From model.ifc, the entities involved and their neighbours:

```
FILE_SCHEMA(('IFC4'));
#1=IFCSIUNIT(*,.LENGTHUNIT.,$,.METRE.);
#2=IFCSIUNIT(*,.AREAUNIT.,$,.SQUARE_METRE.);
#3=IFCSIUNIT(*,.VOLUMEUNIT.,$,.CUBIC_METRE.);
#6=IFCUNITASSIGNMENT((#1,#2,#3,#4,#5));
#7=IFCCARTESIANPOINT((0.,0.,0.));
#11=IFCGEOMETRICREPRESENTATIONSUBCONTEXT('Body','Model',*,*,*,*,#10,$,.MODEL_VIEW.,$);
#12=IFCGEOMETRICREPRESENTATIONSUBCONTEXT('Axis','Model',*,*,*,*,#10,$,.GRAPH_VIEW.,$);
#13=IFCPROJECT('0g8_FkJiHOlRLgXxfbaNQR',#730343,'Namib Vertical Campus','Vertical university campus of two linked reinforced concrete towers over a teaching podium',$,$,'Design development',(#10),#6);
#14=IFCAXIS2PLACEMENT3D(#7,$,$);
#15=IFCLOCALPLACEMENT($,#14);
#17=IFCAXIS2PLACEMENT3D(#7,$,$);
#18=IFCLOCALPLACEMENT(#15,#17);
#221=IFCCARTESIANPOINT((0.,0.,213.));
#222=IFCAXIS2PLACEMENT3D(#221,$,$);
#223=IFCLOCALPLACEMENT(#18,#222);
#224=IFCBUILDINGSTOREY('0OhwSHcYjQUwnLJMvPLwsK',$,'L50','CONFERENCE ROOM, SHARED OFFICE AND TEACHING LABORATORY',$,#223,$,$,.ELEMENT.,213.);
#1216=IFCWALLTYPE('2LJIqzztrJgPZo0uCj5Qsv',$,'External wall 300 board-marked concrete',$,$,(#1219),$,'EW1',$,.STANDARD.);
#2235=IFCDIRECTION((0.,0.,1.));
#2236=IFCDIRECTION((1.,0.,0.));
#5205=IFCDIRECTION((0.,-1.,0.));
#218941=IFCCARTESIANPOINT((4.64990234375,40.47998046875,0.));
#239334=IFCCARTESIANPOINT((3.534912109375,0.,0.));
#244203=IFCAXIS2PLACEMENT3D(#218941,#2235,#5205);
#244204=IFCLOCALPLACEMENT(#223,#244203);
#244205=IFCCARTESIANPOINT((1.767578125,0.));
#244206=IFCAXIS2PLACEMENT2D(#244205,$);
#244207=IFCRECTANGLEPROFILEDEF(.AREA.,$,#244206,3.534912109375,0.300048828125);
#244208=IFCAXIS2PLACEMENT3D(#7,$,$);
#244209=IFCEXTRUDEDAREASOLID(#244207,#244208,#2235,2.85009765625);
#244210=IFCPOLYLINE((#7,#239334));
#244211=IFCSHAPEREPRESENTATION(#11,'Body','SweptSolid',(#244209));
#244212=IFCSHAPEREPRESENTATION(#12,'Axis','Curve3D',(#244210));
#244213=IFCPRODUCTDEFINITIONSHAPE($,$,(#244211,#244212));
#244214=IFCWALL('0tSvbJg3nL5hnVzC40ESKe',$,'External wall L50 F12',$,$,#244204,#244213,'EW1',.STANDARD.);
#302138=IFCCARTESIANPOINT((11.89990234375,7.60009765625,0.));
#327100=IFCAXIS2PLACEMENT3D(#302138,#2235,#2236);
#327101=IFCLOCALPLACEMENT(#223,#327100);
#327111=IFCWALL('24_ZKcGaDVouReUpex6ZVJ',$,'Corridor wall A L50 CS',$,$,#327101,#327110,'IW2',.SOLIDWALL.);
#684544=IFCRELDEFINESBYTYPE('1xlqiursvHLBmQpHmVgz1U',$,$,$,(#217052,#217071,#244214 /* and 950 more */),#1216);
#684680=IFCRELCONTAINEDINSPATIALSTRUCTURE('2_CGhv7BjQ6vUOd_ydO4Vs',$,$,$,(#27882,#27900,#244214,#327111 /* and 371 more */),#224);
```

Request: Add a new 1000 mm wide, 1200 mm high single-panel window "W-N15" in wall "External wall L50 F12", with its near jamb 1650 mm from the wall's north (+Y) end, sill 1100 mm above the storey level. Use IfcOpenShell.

```python
import numpy as np
import ifcopenshell
import ifcopenshell.api.feature
import ifcopenshell.api.geometry
import ifcopenshell.api.root
import ifcopenshell.api.spatial
import ifcopenshell.geom
import ifcopenshell.util.element
import ifcopenshell.util.placement
import ifcopenshell.util.representation
import ifcopenshell.util.shape
import ifcopenshell.util.unit

model = ifcopenshell.open("model.ifc")
unit_scale = ifcopenshell.util.unit.calculate_unit_scale(model)
settings = ifcopenshell.geom.settings()


def volume(element):
    """Net volume in cubic metres, openings subtracted."""
    shape = ifcopenshell.geom.create_shape(settings, element)
    return ifcopenshell.util.shape.get_volume(shape.geometry)


wall = model.by_guid("0tSvbJg3nL5hnVzC40ESKe")
storey = ifcopenshell.util.element.get_container(wall, ifc_class="IfcBuildingStorey")
context = ifcopenshell.util.representation.get_context(model, "Model", "Body", "MODEL_VIEW")
before = volume(wall)

width, height, from_end, sill = 1, 1.2, 1.65, 1.1  # metres

# The wall runs along its own X axis, and the end named is its -X end.
wall_shape = ifcopenshell.geom.create_shape(settings, wall)
x, y, z = ifcopenshell.util.shape.get_vertices(wall_shape.geometry).T
start = x.min() + from_end
face, thickness = float(y.min()), float(y.max() - y.min())
wall_matrix = ifcopenshell.util.placement.get_local_placement(wall.ObjectPlacement)
level = ifcopenshell.util.placement.get_local_placement(storey.ObjectPlacement)[2, 3]


def in_wall(x, y):
    """Placement at x, y metres in the wall's axes, at sill height."""
    matrix = wall_matrix.copy()
    matrix[:, 3] = wall_matrix @ np.array([x / unit_scale, y / unit_scale, 0.0, 1.0])
    matrix[2, 3] = level + sill / unit_scale
    return matrix


# Opening: a box that overshoots both wall faces by 50 mm.
opening = ifcopenshell.api.root.create_entity(model, ifc_class="IfcOpeningElement", predefined_type="OPENING")
box = ifcopenshell.api.geometry.add_wall_representation(
    model, context=context, length=width, height=height, thickness=thickness + 0.1
)
ifcopenshell.api.geometry.assign_representation(model, product=opening, representation=box)
ifcopenshell.api.geometry.edit_object_placement(model, product=opening, matrix=in_wall(start, face - 0.05), is_si=False)
ifcopenshell.api.feature.add_feature(model, feature=opening, element=wall)

window = ifcopenshell.api.root.create_entity(model, ifc_class="IfcWindow", name="W-N15", predefined_type="WINDOW")
window.OverallWidth, window.OverallHeight = width / unit_scale, height / unit_scale
window.PartitioningType = "SINGLE_PANEL"
body = ifcopenshell.api.geometry.add_window_representation(
    model,
    context=context,
    overall_width=window.OverallWidth,
    overall_height=window.OverallHeight,
    partition_type="SINGLE_PANEL",
)
ifcopenshell.api.geometry.assign_representation(model, product=window, representation=body)
ifcopenshell.api.spatial.assign_container(model, products=[window], relating_structure=storey)
ifcopenshell.api.feature.add_filling(model, opening=opening, element=window)

# Centre the window in the wall's thickness.
ifcopenshell.api.geometry.edit_object_placement(model, product=window, matrix=in_wall(start, face), is_si=False)
window_shape = ifcopenshell.geom.create_shape(settings, window)
depth = ifcopenshell.util.shape.get_vertices(window_shape.geometry)[:, 1]
offset = face + thickness / 2 - (depth.min() + depth.max()) / 2
ifcopenshell.api.geometry.edit_object_placement(model, product=window, matrix=in_wall(start, offset), is_si=False)

after = volume(wall)

print(f"wall volume {before:.3f} -> {after:.3f} m3")

model.write("model_v2.ifc")
```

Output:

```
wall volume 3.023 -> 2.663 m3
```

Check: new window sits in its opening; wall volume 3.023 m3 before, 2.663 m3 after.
